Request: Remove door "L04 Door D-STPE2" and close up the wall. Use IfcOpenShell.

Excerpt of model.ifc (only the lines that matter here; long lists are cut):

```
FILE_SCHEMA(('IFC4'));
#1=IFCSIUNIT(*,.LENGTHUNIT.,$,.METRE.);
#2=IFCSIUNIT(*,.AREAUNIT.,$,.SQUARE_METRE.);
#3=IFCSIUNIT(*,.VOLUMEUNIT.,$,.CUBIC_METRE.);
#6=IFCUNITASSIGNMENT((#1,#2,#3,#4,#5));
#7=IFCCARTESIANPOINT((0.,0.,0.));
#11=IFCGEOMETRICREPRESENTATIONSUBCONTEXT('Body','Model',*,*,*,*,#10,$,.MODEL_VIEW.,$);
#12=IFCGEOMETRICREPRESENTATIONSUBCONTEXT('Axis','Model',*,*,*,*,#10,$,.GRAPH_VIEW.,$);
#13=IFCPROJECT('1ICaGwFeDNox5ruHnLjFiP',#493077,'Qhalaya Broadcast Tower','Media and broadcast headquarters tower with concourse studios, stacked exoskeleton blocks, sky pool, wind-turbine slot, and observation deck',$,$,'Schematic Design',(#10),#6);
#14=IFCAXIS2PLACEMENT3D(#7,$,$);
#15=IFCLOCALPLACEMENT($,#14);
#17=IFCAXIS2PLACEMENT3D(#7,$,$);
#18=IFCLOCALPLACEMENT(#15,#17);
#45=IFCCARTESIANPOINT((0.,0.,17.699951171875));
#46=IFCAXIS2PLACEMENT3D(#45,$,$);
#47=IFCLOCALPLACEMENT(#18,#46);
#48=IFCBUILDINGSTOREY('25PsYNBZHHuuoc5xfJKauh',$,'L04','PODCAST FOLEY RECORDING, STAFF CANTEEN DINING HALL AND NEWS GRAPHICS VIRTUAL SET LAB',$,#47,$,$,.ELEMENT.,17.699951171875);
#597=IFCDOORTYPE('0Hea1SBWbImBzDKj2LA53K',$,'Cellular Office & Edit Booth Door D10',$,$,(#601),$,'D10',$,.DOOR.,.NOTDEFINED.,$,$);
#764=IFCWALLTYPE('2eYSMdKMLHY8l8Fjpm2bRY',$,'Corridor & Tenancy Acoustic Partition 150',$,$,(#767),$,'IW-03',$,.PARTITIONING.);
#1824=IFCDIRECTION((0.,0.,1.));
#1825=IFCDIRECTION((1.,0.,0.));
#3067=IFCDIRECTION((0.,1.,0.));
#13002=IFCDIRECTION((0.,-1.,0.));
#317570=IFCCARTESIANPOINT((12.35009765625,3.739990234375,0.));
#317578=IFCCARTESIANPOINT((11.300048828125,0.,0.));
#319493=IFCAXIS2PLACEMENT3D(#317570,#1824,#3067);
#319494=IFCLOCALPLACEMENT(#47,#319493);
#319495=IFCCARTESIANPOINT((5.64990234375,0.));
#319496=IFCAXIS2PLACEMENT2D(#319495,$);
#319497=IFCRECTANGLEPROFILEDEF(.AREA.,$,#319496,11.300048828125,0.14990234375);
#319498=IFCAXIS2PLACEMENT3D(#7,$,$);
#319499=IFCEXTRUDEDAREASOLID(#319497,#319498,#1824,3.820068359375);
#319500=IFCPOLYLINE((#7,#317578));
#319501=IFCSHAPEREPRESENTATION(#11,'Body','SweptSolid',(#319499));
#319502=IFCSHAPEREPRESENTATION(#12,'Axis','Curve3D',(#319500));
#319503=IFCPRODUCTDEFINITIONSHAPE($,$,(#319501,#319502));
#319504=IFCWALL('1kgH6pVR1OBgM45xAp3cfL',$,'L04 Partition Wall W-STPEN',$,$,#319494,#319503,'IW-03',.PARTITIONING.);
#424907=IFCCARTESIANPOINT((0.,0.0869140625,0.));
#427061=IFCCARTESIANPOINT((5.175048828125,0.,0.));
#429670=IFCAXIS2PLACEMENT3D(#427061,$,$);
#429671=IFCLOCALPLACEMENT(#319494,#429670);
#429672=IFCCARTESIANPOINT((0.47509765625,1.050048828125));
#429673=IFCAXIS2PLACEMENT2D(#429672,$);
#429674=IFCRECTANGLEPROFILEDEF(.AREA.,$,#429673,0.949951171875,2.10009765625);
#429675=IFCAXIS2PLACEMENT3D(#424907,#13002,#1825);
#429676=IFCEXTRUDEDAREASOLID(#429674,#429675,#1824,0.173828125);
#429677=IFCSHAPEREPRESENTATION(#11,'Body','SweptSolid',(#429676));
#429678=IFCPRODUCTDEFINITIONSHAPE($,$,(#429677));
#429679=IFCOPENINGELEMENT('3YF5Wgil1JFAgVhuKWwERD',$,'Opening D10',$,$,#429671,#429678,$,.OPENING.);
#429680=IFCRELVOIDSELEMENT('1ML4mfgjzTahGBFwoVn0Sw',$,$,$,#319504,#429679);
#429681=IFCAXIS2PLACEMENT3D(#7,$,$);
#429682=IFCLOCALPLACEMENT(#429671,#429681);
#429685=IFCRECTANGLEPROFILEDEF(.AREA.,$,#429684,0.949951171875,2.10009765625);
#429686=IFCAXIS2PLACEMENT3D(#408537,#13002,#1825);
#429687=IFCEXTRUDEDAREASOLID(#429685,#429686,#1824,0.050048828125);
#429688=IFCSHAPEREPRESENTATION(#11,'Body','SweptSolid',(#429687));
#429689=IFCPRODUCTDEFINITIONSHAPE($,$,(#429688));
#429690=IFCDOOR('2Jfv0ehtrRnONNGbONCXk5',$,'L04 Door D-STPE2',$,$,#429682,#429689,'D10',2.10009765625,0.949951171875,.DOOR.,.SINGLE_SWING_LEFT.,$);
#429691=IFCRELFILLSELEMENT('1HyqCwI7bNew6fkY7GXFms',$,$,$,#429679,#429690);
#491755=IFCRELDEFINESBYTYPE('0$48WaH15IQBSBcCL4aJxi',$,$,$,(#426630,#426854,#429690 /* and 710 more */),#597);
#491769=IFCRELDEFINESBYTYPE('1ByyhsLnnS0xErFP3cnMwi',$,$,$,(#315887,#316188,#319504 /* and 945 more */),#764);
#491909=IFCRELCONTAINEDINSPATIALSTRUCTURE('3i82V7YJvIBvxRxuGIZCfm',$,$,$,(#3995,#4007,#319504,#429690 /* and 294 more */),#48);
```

```python
import ifcopenshell
import ifcopenshell.api.feature
import ifcopenshell.api.root
import ifcopenshell.geom
import ifcopenshell.util.shape

model = ifcopenshell.open("model.ifc")
settings = ifcopenshell.geom.settings()


def volume(element):
    """Net volume in cubic metres, openings subtracted."""
    shape = ifcopenshell.geom.create_shape(settings, element)
    return ifcopenshell.util.shape.get_volume(shape.geometry)


door = model.by_id(429690)
opening = door.FillsVoids[0].RelatingOpeningElement
wall = opening.VoidsElements[0].RelatingBuildingElement
before = volume(wall)

ifcopenshell.api.root.remove_product(model, product=door)
ifcopenshell.api.feature.remove_feature(model, feature=opening)

after = volume(wall)

print(f"wall volume {before:.3f} -> {after:.3f} m3")

model.write("model_updated.ifc")
```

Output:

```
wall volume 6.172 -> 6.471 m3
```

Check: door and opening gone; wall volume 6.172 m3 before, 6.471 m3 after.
